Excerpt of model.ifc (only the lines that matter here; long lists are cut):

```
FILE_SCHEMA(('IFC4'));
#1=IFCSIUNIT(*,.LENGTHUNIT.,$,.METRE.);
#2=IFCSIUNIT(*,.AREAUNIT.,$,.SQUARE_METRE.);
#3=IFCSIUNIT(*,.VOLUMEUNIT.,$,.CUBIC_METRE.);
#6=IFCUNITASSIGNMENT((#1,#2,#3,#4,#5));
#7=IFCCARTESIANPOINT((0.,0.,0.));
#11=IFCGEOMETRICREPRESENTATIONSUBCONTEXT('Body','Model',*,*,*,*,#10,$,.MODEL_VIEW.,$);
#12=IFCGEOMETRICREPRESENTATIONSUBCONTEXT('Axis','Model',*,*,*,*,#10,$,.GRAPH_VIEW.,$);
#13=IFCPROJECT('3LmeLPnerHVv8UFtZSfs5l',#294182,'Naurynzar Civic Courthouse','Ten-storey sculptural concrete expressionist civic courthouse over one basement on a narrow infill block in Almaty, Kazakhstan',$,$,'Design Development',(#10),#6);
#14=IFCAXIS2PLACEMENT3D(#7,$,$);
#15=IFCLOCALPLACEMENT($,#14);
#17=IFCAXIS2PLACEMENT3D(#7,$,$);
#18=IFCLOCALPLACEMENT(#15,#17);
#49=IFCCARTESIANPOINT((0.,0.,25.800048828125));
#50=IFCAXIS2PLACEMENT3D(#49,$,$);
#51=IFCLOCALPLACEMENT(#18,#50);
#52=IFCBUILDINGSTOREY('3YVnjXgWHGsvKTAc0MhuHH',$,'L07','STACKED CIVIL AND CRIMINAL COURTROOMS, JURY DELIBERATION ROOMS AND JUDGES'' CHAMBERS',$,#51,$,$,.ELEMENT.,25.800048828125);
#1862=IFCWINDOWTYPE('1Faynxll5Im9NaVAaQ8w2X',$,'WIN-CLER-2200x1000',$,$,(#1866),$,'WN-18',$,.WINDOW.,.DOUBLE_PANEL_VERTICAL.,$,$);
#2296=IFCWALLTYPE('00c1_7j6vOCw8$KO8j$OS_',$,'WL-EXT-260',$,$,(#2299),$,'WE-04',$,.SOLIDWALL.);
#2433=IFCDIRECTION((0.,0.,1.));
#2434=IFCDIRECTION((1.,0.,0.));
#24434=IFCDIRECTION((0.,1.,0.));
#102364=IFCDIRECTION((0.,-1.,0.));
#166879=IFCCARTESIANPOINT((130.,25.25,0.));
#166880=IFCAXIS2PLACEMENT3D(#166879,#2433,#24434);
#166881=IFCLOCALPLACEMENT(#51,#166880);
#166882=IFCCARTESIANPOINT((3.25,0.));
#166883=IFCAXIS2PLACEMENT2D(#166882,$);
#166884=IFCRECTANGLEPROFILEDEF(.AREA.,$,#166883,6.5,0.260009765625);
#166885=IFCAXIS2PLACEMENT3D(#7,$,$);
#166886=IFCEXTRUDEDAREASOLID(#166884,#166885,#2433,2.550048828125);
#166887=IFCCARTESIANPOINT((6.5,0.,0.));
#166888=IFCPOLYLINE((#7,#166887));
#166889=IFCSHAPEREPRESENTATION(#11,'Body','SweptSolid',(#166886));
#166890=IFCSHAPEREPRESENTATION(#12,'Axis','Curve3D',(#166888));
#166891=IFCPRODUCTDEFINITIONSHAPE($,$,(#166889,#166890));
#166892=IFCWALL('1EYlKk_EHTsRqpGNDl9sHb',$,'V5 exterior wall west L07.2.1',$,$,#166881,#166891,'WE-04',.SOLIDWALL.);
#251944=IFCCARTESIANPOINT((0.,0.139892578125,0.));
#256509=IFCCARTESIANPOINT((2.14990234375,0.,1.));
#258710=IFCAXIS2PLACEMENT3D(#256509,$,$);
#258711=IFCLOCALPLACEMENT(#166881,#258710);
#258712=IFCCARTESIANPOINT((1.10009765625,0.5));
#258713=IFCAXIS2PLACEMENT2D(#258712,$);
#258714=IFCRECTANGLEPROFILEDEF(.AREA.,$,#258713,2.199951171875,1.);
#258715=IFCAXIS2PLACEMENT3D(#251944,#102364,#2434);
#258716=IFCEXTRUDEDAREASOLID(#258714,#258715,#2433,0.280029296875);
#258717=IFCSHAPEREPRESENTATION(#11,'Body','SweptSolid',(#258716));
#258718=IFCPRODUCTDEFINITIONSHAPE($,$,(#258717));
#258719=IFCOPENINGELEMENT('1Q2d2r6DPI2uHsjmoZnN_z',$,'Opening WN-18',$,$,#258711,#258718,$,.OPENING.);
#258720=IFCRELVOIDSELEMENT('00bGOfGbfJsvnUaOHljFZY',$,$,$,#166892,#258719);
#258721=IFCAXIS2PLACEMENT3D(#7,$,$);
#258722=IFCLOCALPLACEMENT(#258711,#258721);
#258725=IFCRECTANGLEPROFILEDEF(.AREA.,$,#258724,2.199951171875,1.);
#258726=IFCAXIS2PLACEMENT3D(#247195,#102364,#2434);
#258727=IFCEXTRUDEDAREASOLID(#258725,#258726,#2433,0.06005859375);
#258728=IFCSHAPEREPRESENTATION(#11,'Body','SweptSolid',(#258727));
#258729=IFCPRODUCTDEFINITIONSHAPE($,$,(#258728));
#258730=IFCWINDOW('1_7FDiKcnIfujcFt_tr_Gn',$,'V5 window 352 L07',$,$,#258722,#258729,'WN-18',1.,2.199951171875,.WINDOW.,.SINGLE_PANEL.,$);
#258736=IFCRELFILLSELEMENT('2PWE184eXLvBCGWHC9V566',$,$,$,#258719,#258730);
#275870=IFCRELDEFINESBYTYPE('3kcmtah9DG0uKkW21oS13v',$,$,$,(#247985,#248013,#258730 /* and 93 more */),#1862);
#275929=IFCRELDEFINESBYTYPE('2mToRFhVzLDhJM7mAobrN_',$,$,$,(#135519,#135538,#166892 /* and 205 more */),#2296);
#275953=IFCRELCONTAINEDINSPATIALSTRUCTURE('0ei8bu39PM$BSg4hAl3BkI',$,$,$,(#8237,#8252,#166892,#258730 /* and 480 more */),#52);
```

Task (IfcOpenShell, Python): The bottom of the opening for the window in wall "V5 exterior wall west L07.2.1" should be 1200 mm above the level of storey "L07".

```python
import numpy as np
import ifcopenshell
import ifcopenshell.api.geometry
import ifcopenshell.geom
import ifcopenshell.util.element
import ifcopenshell.util.placement
import ifcopenshell.util.shape
import ifcopenshell.util.unit

model = ifcopenshell.open("model.ifc")
unit_scale = ifcopenshell.util.unit.calculate_unit_scale(model)

window = model.by_guid("1_7FDiKcnIfujcFt_tr_Gn")
opening = window.FillsVoids[0].RelatingOpeningElement
storey = ifcopenshell.util.element.get_container(window, ifc_class="IfcBuildingStorey")
level = ifcopenshell.util.placement.get_local_placement(storey.ObjectPlacement)[2, 3]

# The opening's origin need not be at the sill, so measure its lowest point.
shape = ifcopenshell.geom.create_shape(ifcopenshell.geom.settings(), opening)
bottom = ifcopenshell.util.shape.get_shape_bottom_elevation(shape, shape.geometry) / unit_scale
dz = level + 1.2 - bottom

shift = np.array([0.0, 0.0, dz])
# The window is placed relative to its opening, so it follows when the opening moves.
matrix = ifcopenshell.util.placement.get_local_placement(opening.ObjectPlacement)
matrix[:3, 3] += shift
ifcopenshell.api.geometry.edit_object_placement(
    model, product=opening, matrix=matrix, is_si=False, should_transform_children=True
)

print(f"moved by {dz * unit_scale:+.3f} m")

model.write("model_updated.ifc")
```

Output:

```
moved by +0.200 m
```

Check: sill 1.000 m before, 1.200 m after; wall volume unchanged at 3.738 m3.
